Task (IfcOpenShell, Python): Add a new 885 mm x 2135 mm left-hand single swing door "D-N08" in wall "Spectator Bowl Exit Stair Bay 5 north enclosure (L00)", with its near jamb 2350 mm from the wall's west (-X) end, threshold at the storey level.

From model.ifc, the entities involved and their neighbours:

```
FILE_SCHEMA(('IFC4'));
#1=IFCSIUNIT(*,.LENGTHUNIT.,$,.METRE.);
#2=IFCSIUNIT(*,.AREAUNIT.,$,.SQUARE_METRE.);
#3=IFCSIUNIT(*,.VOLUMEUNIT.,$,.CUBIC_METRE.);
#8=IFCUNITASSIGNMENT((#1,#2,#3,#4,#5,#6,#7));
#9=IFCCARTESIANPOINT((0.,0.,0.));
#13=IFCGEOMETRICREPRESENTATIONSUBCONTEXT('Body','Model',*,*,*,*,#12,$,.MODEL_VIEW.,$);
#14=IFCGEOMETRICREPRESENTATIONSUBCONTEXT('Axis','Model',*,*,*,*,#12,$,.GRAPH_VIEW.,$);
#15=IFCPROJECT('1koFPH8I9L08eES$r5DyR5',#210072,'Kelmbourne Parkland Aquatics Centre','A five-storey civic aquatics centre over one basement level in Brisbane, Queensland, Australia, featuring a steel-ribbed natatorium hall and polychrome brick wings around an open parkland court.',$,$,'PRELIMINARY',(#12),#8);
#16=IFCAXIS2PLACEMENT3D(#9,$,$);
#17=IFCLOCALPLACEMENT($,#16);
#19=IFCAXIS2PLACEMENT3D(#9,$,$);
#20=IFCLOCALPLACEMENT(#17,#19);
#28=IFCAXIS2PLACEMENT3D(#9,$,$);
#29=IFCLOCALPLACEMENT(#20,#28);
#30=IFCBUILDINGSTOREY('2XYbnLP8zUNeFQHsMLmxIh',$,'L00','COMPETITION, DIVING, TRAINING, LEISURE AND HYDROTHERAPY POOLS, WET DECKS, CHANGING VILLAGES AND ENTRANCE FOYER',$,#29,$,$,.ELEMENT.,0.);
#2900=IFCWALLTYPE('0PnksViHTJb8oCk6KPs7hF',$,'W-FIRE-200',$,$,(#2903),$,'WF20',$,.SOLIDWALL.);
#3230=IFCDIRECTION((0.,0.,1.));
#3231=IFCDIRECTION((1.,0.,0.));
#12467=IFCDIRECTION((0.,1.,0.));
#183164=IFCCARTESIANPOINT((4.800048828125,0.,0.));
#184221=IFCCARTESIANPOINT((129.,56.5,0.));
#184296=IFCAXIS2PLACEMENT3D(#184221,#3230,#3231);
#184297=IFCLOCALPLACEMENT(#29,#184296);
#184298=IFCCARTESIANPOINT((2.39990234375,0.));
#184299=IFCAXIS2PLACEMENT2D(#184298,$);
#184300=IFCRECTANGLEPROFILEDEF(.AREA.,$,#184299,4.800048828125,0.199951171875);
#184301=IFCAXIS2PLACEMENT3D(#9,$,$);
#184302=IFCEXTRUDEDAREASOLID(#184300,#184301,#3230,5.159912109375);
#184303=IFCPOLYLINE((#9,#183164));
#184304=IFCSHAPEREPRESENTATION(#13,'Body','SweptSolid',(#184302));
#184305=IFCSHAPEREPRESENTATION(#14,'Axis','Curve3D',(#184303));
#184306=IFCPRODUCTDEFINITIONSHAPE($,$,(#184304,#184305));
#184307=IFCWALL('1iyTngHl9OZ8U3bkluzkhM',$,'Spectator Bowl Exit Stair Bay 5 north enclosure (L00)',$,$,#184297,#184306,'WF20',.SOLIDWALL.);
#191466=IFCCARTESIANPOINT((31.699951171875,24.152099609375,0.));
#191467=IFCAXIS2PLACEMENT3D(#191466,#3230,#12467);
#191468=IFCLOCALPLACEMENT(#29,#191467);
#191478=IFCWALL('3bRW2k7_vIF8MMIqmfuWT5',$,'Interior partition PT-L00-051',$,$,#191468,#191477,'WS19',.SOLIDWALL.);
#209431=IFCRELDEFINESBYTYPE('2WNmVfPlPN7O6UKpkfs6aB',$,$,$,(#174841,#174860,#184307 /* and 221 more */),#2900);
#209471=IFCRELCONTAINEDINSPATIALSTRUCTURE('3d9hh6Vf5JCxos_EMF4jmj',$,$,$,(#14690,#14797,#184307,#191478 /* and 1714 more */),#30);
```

```python
import numpy as np
import ifcopenshell
import ifcopenshell.api.feature
import ifcopenshell.api.geometry
import ifcopenshell.api.root
import ifcopenshell.api.spatial
import ifcopenshell.geom
import ifcopenshell.util.element
import ifcopenshell.util.placement
import ifcopenshell.util.representation
import ifcopenshell.util.shape
import ifcopenshell.util.unit

model = ifcopenshell.open("model.ifc")
unit_scale = ifcopenshell.util.unit.calculate_unit_scale(model)
settings = ifcopenshell.geom.settings()


def volume(element):
    """Net volume in cubic metres, openings subtracted."""
    shape = ifcopenshell.geom.create_shape(settings, element)
    return ifcopenshell.util.shape.get_volume(shape.geometry)


wall = model.by_guid("1iyTngHl9OZ8U3bkluzkhM")
storey = ifcopenshell.util.element.get_container(wall, ifc_class="IfcBuildingStorey")
context = ifcopenshell.util.representation.get_context(model, "Model", "Body", "MODEL_VIEW")
before = volume(wall)

width, height, from_end, sill = 0.885, 2.135, 2.35, 0.0  # metres

# The wall runs along its own X axis, and the end named is its -X end.
wall_shape = ifcopenshell.geom.create_shape(settings, wall)
x, y, z = ifcopenshell.util.shape.get_vertices(wall_shape.geometry).T
start = x.min() + from_end
face, thickness = float(y.min()), float(y.max() - y.min())
wall_matrix = ifcopenshell.util.placement.get_local_placement(wall.ObjectPlacement)
level = ifcopenshell.util.placement.get_local_placement(storey.ObjectPlacement)[2, 3]


def in_wall(x, y):
    """Placement at x, y metres in the wall's axes, at sill height."""
    matrix = wall_matrix.copy()
    matrix[:, 3] = wall_matrix @ np.array([x / unit_scale, y / unit_scale, 0.0, 1.0])
    matrix[2, 3] = level + sill / unit_scale
    return matrix


# Opening: a box that overshoots both wall faces by 50 mm.
opening = ifcopenshell.api.root.create_entity(model, ifc_class="IfcOpeningElement", predefined_type="OPENING")
box = ifcopenshell.api.geometry.add_wall_representation(
    model, context=context, length=width, height=height, thickness=thickness + 0.1
)
ifcopenshell.api.geometry.assign_representation(model, product=opening, representation=box)
ifcopenshell.api.geometry.edit_object_placement(model, product=opening, matrix=in_wall(start, face - 0.05), is_si=False)
ifcopenshell.api.feature.add_feature(model, feature=opening, element=wall)

door = ifcopenshell.api.root.create_entity(model, ifc_class="IfcDoor", name="D-N08", predefined_type="DOOR")
door.OverallWidth, door.OverallHeight = width / unit_scale, height / unit_scale
door.OperationType = "SINGLE_SWING_LEFT"
body = ifcopenshell.api.geometry.add_door_representation(
    model,
    context=context,
    overall_width=door.OverallWidth,
    overall_height=door.OverallHeight,
    operation_type="SINGLE_SWING_LEFT",
    lining_properties={"LiningDepth": thickness / unit_scale, "ThresholdDepth": thickness / unit_scale},
)
ifcopenshell.api.geometry.assign_representation(model, product=door, representation=body)
ifcopenshell.api.spatial.assign_container(model, products=[door], relating_structure=storey)
ifcopenshell.api.feature.add_filling(model, opening=opening, element=door)

# The lining spans the wall, so the door starts at the wall face.
ifcopenshell.api.geometry.edit_object_placement(model, product=door, matrix=in_wall(start, face), is_si=False)

after = volume(wall)

print(f"wall volume {before:.3f} -> {after:.3f} m3")

model.write("model_v2.ifc")
```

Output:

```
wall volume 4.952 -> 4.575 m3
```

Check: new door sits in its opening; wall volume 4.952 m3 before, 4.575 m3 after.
